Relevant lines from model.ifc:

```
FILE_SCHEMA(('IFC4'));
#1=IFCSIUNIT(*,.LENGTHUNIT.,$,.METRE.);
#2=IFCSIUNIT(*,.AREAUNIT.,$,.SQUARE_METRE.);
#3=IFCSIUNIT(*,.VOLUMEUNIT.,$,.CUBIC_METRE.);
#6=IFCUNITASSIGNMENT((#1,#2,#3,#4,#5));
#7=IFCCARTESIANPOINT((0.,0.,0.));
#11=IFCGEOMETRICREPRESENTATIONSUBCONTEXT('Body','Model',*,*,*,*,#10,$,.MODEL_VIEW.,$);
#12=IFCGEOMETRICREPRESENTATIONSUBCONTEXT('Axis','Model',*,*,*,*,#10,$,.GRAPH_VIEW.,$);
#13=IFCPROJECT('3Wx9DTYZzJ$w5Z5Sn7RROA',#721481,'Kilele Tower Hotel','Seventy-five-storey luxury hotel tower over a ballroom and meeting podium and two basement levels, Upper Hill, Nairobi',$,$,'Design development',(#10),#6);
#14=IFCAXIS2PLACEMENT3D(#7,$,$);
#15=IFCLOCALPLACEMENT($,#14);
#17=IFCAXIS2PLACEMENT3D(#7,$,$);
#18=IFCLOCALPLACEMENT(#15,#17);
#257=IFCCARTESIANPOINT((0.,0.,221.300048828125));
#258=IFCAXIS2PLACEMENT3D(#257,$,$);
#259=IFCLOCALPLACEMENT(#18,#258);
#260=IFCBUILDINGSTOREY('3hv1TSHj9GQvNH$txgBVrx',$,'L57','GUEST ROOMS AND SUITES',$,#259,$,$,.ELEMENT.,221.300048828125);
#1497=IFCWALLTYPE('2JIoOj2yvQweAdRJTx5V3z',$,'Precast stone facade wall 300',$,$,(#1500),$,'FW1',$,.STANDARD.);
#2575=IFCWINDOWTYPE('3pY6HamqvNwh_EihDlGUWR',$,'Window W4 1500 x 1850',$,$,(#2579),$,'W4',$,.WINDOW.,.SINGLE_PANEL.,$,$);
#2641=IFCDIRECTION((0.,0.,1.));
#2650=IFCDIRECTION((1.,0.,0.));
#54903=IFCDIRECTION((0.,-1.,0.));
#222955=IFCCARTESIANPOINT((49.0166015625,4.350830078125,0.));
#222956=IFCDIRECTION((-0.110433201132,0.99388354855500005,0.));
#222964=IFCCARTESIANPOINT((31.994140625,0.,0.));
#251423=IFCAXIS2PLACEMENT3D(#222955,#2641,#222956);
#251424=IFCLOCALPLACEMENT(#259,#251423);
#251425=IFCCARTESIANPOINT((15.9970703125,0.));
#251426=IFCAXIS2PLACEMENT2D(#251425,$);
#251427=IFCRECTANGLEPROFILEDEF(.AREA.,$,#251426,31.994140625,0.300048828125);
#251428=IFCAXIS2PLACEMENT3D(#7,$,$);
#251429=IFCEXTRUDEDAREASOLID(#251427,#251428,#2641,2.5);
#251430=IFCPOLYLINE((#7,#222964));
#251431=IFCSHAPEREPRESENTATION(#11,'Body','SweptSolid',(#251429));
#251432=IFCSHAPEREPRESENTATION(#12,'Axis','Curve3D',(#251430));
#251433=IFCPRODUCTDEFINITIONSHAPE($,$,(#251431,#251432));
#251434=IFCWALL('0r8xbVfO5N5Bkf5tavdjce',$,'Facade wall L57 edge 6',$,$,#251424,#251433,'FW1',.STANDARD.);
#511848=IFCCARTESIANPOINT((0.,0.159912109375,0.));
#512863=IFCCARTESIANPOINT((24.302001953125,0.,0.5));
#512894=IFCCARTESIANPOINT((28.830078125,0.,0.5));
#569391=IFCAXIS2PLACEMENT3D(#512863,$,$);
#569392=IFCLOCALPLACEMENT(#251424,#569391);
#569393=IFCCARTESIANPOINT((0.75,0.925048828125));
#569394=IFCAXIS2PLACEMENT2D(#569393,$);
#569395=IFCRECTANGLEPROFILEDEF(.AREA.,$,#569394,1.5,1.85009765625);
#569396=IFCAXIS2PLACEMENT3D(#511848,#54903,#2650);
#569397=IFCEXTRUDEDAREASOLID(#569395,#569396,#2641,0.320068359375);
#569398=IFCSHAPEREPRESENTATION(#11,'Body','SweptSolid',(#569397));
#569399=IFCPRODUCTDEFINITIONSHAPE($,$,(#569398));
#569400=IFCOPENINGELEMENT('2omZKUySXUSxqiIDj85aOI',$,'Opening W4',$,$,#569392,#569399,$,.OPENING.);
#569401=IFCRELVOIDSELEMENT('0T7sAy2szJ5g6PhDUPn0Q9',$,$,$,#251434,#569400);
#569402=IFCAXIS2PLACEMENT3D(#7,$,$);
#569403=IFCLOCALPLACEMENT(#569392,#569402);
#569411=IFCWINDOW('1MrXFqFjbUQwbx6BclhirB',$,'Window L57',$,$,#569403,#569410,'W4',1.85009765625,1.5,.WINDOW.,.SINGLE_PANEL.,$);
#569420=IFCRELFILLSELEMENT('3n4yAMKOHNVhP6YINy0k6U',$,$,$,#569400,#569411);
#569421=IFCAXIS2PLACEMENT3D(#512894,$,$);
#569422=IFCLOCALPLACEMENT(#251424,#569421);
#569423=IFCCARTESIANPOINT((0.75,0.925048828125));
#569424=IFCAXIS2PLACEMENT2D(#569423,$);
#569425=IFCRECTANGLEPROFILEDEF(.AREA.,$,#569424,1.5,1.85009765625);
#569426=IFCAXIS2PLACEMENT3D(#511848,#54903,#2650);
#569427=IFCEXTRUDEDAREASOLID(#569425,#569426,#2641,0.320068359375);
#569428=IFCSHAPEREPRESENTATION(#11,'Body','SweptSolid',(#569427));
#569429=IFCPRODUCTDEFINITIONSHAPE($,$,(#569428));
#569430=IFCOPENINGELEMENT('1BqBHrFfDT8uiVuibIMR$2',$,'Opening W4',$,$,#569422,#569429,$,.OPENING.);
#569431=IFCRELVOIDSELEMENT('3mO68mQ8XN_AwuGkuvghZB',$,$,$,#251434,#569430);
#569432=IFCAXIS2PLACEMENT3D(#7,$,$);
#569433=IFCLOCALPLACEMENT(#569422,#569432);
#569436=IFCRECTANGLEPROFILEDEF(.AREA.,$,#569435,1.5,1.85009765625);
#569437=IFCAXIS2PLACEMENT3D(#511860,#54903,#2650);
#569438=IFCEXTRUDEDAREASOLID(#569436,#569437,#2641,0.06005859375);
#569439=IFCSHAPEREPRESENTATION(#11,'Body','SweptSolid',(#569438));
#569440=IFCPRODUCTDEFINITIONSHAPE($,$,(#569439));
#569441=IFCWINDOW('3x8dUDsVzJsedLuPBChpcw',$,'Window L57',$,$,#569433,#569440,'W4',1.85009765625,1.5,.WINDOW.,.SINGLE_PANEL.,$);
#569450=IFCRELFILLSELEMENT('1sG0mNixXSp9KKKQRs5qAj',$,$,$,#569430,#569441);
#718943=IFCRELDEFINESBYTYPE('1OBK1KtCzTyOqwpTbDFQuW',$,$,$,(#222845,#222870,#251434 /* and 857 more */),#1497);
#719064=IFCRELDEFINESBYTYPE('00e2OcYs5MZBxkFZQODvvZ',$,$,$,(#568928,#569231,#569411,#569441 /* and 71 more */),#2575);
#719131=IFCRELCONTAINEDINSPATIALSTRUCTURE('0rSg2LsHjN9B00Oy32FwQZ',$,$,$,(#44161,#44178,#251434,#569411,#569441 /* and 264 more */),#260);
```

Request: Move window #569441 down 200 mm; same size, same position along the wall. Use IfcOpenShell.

```python
import numpy as np
import ifcopenshell
import ifcopenshell.api.geometry
import ifcopenshell.util.placement
import ifcopenshell.util.unit

model = ifcopenshell.open("model.ifc")
unit_scale = ifcopenshell.util.unit.calculate_unit_scale(model)

window = model.by_id(569441)
opening = window.FillsVoids[0].RelatingOpeningElement
dz = -0.2

shift = np.array([0.0, 0.0, dz])
# The window is placed relative to its opening, so it follows when the opening moves.
matrix = ifcopenshell.util.placement.get_local_placement(opening.ObjectPlacement)
matrix[:3, 3] += shift
ifcopenshell.api.geometry.edit_object_placement(
    model, product=opening, matrix=matrix, is_si=False, should_transform_children=True
)

print(f"moved by {dz * unit_scale:+.3f} m")

model.write("model_edited.ifc")
```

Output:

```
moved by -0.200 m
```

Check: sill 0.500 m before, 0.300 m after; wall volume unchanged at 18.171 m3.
